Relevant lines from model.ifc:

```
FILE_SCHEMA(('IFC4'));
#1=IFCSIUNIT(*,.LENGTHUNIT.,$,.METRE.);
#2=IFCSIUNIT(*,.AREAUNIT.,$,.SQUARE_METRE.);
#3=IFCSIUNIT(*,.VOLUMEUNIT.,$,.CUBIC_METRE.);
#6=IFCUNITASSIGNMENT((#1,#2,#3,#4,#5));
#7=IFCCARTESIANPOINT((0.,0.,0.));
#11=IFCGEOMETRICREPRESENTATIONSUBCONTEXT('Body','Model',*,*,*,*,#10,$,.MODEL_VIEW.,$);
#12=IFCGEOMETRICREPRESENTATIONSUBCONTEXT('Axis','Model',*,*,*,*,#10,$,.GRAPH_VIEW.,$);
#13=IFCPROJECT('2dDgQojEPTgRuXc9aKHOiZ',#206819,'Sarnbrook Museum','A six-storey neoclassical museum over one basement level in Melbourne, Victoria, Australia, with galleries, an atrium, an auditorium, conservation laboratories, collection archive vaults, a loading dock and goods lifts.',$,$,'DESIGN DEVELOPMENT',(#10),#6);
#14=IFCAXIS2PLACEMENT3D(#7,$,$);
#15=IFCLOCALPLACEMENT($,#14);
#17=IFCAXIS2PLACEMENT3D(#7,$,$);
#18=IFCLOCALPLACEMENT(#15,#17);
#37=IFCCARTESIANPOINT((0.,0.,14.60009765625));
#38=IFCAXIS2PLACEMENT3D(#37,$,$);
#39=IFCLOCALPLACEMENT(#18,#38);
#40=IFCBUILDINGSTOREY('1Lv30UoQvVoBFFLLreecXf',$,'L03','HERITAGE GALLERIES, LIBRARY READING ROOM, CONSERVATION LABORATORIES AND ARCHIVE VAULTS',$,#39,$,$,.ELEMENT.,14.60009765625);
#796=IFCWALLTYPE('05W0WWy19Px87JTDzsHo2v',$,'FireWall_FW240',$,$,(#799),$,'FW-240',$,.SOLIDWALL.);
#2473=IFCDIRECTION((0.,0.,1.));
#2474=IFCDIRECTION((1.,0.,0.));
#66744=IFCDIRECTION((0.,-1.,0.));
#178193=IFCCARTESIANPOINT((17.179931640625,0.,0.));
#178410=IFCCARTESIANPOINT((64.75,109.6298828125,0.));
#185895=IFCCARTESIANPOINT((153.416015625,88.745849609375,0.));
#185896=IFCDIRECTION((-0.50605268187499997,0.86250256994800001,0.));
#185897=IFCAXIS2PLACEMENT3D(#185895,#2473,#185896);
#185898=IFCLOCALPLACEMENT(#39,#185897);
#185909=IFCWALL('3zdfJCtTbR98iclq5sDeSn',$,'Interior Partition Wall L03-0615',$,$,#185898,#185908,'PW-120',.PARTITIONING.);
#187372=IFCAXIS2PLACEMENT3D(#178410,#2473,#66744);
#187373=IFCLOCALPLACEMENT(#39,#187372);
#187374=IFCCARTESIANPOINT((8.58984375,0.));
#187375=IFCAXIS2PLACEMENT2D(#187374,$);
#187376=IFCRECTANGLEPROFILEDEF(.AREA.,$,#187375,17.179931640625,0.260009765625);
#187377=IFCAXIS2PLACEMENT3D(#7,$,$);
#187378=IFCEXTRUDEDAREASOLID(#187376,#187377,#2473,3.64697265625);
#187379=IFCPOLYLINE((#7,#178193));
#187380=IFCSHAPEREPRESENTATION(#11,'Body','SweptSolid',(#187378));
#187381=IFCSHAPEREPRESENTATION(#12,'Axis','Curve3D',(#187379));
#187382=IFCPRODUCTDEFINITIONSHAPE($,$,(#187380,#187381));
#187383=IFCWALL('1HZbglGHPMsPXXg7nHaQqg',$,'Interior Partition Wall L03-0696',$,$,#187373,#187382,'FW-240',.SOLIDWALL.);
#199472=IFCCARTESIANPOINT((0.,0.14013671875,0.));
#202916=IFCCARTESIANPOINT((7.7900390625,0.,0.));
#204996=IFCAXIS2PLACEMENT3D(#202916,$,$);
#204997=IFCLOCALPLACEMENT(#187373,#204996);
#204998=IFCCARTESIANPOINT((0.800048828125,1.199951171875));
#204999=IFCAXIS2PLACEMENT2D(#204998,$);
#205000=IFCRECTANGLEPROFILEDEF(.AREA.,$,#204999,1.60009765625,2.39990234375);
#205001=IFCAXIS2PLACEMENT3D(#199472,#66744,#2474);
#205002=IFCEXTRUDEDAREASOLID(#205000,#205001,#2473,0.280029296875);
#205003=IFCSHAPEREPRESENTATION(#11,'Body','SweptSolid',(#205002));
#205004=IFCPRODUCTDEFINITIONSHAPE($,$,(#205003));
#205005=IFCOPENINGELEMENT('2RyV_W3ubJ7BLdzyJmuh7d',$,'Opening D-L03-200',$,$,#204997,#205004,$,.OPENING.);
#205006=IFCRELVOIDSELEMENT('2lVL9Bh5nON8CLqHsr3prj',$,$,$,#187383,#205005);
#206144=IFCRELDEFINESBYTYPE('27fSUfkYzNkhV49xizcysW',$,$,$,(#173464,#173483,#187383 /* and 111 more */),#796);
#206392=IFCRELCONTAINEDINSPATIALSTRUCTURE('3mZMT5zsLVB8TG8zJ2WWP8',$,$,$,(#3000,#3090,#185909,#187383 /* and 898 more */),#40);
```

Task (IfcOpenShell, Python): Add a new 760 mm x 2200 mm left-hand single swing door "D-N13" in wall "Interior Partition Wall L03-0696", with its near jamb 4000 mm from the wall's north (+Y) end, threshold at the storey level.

```python
import numpy as np
import ifcopenshell
import ifcopenshell.api.feature
import ifcopenshell.api.geometry
import ifcopenshell.api.root
import ifcopenshell.api.spatial
import ifcopenshell.geom
import ifcopenshell.util.element
import ifcopenshell.util.placement
import ifcopenshell.util.representation
import ifcopenshell.util.shape
import ifcopenshell.util.unit

model = ifcopenshell.open("model.ifc")
unit_scale = ifcopenshell.util.unit.calculate_unit_scale(model)
settings = ifcopenshell.geom.settings()


def volume(element):
    """Net volume in cubic metres, openings subtracted."""
    shape = ifcopenshell.geom.create_shape(settings, element)
    return ifcopenshell.util.shape.get_volume(shape.geometry)


wall = model.by_id(187383)
storey = ifcopenshell.util.element.get_container(wall, ifc_class="IfcBuildingStorey")
context = ifcopenshell.util.representation.get_context(model, "Model", "Body", "MODEL_VIEW")
before = volume(wall)

width, height, from_end, sill = 0.76, 2.2, 4, 0.0  # metres

# The wall runs along its own X axis, and the end named is its -X end.
wall_shape = ifcopenshell.geom.create_shape(settings, wall)
x, y, z = ifcopenshell.util.shape.get_vertices(wall_shape.geometry).T
start = x.min() + from_end
face, thickness = float(y.min()), float(y.max() - y.min())
wall_matrix = ifcopenshell.util.placement.get_local_placement(wall.ObjectPlacement)
level = ifcopenshell.util.placement.get_local_placement(storey.ObjectPlacement)[2, 3]


def in_wall(x, y):
    """Placement at x, y metres in the wall's axes, at sill height."""
    matrix = wall_matrix.copy()
    matrix[:, 3] = wall_matrix @ np.array([x / unit_scale, y / unit_scale, 0.0, 1.0])
    matrix[2, 3] = level + sill / unit_scale
    return matrix


# Opening: a box that overshoots both wall faces by 50 mm.
opening = ifcopenshell.api.root.create_entity(model, ifc_class="IfcOpeningElement", predefined_type="OPENING")
box = ifcopenshell.api.geometry.add_wall_representation(
    model, context=context, length=width, height=height, thickness=thickness + 0.1
)
ifcopenshell.api.geometry.assign_representation(model, product=opening, representation=box)
ifcopenshell.api.geometry.edit_object_placement(model, product=opening, matrix=in_wall(start, face - 0.05), is_si=False)
ifcopenshell.api.feature.add_feature(model, feature=opening, element=wall)

door = ifcopenshell.api.root.create_entity(model, ifc_class="IfcDoor", name="D-N13", predefined_type="DOOR")
door.OverallWidth, door.OverallHeight = width / unit_scale, height / unit_scale
door.OperationType = "SINGLE_SWING_LEFT"
body = ifcopenshell.api.geometry.add_door_representation(
    model,
    context=context,
    overall_width=door.OverallWidth,
    overall_height=door.OverallHeight,
    operation_type="SINGLE_SWING_LEFT",
    lining_properties={"LiningDepth": thickness / unit_scale, "ThresholdDepth": thickness / unit_scale},
)
ifcopenshell.api.geometry.assign_representation(model, product=door, representation=body)
ifcopenshell.api.spatial.assign_container(model, products=[door], relating_structure=storey)
ifcopenshell.api.feature.add_filling(model, opening=opening, element=door)

# The lining spans the wall, so the door starts at the wall face.
ifcopenshell.api.geometry.edit_object_placement(model, product=door, matrix=in_wall(start, face), is_si=False)

after = volume(wall)

print(f"wall volume {before:.3f} -> {after:.3f} m3")

model.write("model_updated.ifc")
```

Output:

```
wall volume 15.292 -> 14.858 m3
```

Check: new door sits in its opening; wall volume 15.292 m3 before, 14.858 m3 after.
